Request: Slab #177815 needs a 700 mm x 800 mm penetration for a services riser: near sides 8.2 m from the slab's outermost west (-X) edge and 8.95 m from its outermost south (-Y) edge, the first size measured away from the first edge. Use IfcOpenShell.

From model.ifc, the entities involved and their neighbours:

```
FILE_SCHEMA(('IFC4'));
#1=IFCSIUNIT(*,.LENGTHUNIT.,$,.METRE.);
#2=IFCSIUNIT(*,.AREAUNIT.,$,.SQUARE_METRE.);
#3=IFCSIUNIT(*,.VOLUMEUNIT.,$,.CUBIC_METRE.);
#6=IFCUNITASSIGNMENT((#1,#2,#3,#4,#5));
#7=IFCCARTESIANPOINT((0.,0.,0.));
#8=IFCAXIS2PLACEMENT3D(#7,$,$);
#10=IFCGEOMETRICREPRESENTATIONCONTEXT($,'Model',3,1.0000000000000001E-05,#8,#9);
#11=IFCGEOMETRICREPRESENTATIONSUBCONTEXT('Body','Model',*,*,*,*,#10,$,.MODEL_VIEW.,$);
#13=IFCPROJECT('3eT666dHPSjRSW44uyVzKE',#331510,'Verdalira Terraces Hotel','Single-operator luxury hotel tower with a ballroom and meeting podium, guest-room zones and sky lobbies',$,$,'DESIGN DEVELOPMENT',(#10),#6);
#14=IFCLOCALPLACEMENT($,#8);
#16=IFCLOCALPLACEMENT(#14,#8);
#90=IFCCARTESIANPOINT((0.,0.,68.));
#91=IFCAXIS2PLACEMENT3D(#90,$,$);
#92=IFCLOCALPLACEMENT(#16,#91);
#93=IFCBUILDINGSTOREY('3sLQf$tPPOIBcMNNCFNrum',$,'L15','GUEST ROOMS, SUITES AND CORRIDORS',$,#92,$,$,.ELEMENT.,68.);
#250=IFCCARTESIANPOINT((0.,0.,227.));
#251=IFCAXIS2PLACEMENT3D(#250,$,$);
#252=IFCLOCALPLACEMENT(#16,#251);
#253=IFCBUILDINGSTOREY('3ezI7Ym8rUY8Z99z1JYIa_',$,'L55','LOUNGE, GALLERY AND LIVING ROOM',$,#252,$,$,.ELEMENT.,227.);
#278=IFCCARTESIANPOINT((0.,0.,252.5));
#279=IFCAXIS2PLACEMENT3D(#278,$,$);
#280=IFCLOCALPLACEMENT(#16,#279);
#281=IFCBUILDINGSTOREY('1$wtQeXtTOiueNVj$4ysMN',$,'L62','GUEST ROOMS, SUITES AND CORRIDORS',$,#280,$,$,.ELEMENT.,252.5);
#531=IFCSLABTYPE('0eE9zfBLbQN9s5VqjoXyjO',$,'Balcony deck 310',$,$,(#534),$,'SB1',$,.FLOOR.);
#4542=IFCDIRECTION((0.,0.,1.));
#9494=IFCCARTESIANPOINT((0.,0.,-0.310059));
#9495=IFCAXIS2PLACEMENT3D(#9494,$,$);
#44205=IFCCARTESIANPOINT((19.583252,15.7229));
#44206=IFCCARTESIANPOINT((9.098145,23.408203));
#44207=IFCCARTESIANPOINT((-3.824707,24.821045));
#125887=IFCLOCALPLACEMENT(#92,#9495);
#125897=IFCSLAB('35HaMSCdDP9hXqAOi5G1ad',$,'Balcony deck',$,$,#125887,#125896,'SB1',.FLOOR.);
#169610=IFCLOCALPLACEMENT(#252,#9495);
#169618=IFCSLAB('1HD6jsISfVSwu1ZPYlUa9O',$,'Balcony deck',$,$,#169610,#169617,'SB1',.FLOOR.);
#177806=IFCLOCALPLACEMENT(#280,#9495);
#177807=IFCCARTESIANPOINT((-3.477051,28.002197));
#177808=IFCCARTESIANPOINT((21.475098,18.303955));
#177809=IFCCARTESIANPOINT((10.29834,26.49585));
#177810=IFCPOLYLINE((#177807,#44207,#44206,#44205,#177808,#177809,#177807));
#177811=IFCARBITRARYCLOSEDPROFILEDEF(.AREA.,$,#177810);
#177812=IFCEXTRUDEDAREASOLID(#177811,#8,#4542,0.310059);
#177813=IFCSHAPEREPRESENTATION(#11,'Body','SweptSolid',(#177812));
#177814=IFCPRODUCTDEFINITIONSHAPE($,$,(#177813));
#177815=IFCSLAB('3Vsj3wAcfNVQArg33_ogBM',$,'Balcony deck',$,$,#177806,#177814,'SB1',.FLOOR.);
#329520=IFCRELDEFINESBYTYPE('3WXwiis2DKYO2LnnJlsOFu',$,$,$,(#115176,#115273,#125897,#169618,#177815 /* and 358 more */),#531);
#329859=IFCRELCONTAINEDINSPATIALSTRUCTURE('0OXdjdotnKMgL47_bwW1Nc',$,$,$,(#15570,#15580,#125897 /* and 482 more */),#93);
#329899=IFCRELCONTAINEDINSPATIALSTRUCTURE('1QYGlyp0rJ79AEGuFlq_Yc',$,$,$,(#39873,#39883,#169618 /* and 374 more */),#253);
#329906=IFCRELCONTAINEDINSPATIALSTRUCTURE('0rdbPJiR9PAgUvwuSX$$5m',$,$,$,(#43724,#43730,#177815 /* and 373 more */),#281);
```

```python
import numpy as np
import ifcopenshell
import ifcopenshell.api.feature
import ifcopenshell.api.geometry
import ifcopenshell.api.root
import ifcopenshell.geom
import ifcopenshell.util.placement
import ifcopenshell.util.representation
import ifcopenshell.util.shape
import ifcopenshell.util.unit

model = ifcopenshell.open("model.ifc")
unit_scale = ifcopenshell.util.unit.calculate_unit_scale(model)
settings = ifcopenshell.geom.settings()


def volume(element):
    """Net volume in cubic metres, openings subtracted."""
    shape = ifcopenshell.geom.create_shape(settings, element)
    return ifcopenshell.util.shape.get_volume(shape.geometry)


slab = model.by_guid("3Vsj3wAcfNVQArg33_ogBM")
before = volume(slab)

# Extent in the slab's own axes, in metres. The edges named are its -X and -Y sides.
slab_shape = ifcopenshell.geom.create_shape(settings, slab)
vertices = ifcopenshell.util.shape.get_vertices(slab_shape.geometry)
x_min, y_min, bottom = vertices.min(axis=0)
top = vertices[:, 2].max()

opening = ifcopenshell.api.root.create_entity(model, ifc_class="IfcOpeningElement", name="Services riser opening", predefined_type="OPENING")
context = ifcopenshell.util.representation.get_context(model, "Model", "Body", "MODEL_VIEW")
width, depth = 0.7, 0.8
outline = [(0.0, 0.0), (width, 0.0), (width, depth), (0.0, depth), (0.0, 0.0)]
# Overshoot both faces by 50 mm so the cut is clean.
shape = ifcopenshell.api.geometry.add_slab_representation(
    model, context=context, depth=top - bottom + 0.1, polyline=outline
)
ifcopenshell.api.geometry.assign_representation(model, product=opening, representation=shape)

matrix = ifcopenshell.util.placement.get_local_placement(slab.ObjectPlacement)
matrix[:, 3] = matrix @ np.append(np.array([x_min + 8.2, y_min + 8.95, bottom - 0.05]) / unit_scale, 1.0)
ifcopenshell.api.geometry.edit_object_placement(model, product=opening, matrix=matrix, is_si=False)
ifcopenshell.api.feature.add_feature(model, feature=opening, element=slab)

after = volume(slab)

print(f"slab volume {before:.3f} -> {after:.3f} m3")

model.write("model_edited.ifc")
```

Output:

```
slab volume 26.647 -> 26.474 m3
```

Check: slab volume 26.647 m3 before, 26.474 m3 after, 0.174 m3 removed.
